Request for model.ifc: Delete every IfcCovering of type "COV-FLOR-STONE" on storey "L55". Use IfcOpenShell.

First a look at what the model holds.

```python
import ifcopenshell
import ifcopenshell.util.element

model = ifcopenshell.open("model.ifc")
print(model.schema)
storey = next(s for s in model.by_type("IfcBuildingStorey") if s.Name == "L55")
coverings = [e for e in ifcopenshell.util.element.get_decomposition(storey) if e.is_a("IfcCovering")]
seen = {}
for e in coverings:
    element_type = ifcopenshell.util.element.get_type(e)
    name = element_type.Name if element_type not in (None, e) else None
    seen[name] = seen.get(name, 0) + 1
for name, count in sorted(seen.items(), key=str):
    print(count, "x", name)
```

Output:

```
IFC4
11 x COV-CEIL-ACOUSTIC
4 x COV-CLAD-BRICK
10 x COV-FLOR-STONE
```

```python
import ifcopenshell
import ifcopenshell.api.root
import ifcopenshell.util.element

model = ifcopenshell.open("model.ifc")

storey = next(s for s in model.by_type("IfcBuildingStorey") if s.Name == "L55")
coverings = [e for e in ifcopenshell.util.element.get_decomposition(storey) if e.is_a("IfcCovering")]
targets = [e for e in coverings if (t := ifcopenshell.util.element.get_type(e)) not in (None, e) and t.Name == "COV-FLOR-STONE"]

for e in targets:
    ifcopenshell.api.root.remove_product(model, product=e)
print(len(targets), "removed")

model.write("model-out.ifc")
```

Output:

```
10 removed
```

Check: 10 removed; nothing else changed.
